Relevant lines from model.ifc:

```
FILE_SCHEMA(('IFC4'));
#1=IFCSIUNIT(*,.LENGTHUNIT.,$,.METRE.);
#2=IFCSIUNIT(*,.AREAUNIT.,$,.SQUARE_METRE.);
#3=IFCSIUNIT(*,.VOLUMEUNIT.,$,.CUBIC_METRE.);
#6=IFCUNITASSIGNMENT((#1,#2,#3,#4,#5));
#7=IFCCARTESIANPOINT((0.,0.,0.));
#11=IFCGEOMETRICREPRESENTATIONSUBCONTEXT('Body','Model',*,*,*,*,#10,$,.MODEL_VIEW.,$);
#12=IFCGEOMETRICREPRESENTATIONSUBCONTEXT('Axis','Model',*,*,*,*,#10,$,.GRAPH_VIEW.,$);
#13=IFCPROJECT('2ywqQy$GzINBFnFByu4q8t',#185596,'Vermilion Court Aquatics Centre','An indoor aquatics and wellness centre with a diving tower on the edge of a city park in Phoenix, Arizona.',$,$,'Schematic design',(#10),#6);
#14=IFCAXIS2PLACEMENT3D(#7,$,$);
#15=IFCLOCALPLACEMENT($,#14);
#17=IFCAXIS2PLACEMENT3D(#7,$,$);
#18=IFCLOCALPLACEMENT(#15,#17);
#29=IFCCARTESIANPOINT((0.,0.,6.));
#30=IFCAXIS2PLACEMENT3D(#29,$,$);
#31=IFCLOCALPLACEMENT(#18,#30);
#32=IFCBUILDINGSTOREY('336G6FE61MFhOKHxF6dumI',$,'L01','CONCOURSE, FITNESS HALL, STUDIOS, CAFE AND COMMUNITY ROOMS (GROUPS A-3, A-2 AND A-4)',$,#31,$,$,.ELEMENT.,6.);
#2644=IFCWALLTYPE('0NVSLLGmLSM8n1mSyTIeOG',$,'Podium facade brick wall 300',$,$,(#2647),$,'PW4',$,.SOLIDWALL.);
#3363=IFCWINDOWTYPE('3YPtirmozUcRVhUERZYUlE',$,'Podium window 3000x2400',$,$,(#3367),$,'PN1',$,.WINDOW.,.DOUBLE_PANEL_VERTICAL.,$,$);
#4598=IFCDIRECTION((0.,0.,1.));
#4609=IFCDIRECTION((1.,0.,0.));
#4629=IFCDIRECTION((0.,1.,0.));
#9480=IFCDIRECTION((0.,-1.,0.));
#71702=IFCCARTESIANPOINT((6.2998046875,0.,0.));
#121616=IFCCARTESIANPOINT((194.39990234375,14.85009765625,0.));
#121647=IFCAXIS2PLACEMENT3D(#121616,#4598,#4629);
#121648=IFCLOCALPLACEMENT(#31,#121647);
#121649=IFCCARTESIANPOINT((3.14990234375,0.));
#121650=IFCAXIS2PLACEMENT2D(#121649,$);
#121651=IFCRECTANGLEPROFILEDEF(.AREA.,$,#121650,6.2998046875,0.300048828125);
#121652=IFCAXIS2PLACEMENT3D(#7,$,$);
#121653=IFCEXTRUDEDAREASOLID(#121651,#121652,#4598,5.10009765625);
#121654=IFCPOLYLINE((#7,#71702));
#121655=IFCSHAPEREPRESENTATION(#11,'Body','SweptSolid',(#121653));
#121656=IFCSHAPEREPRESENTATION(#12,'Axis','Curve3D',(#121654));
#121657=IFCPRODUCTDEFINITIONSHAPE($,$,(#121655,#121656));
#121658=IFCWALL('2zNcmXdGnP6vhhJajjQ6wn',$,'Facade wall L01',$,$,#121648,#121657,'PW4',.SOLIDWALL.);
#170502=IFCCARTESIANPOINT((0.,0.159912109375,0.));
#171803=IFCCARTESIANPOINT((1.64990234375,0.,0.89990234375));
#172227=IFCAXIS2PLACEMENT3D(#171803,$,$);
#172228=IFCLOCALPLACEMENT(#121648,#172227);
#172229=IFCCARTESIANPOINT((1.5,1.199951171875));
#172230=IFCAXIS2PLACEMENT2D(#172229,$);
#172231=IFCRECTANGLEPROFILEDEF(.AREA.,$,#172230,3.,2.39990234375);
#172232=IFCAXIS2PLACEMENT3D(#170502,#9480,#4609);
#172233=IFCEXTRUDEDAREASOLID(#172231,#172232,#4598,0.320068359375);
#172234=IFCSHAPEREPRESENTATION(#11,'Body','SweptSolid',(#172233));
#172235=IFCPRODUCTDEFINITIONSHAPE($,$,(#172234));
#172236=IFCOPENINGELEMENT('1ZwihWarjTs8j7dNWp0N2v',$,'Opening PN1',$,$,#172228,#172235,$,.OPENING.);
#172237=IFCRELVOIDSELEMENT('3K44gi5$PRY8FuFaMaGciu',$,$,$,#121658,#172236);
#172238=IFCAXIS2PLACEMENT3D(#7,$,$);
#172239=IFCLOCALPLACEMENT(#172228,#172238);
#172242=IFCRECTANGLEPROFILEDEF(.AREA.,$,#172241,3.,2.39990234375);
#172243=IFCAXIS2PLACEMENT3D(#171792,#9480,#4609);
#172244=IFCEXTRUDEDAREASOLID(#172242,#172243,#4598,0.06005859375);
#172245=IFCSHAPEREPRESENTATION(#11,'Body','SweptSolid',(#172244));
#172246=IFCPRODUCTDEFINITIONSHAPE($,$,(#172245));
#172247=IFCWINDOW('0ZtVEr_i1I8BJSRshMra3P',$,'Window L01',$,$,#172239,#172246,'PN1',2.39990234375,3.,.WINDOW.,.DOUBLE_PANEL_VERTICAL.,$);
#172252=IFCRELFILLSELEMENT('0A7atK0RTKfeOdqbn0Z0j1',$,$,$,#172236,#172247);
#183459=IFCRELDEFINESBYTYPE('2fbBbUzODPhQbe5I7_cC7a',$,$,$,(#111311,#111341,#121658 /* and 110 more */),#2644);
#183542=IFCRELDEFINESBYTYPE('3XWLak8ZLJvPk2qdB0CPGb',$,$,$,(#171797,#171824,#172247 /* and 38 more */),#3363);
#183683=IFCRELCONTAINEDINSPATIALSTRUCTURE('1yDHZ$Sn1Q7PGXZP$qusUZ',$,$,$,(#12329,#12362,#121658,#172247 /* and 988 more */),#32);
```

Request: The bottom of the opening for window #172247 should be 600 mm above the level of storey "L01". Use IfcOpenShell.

```python
import numpy as np
import ifcopenshell
import ifcopenshell.api.geometry
import ifcopenshell.geom
import ifcopenshell.util.element
import ifcopenshell.util.placement
import ifcopenshell.util.shape
import ifcopenshell.util.unit

model = ifcopenshell.open("model.ifc")
unit_scale = ifcopenshell.util.unit.calculate_unit_scale(model)

window = model.by_id(172247)
opening = window.FillsVoids[0].RelatingOpeningElement
storey = ifcopenshell.util.element.get_container(window, ifc_class="IfcBuildingStorey")
level = ifcopenshell.util.placement.get_local_placement(storey.ObjectPlacement)[2, 3]

# The opening's origin need not be at the sill, so measure its lowest point.
shape = ifcopenshell.geom.create_shape(ifcopenshell.geom.settings(), opening)
bottom = ifcopenshell.util.shape.get_shape_bottom_elevation(shape, shape.geometry) / unit_scale
dz = level + 0.6 / unit_scale - bottom

shift = np.array([0.0, 0.0, dz])
# The window is placed relative to its opening, so it follows when the opening moves.
matrix = ifcopenshell.util.placement.get_local_placement(opening.ObjectPlacement)
matrix[:3, 3] += shift
ifcopenshell.api.geometry.edit_object_placement(
    model, product=opening, matrix=matrix, is_si=False, should_transform_children=True
)

print(f"moved by {dz * unit_scale:+.3f} m")

model.write("model_edited.ifc")
```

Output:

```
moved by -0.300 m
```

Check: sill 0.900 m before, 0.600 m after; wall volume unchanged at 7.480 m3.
